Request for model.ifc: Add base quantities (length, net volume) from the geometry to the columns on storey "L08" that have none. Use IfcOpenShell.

First a look at what the model holds.

```python
import ifcopenshell
import ifcopenshell.util.element
import ifcopenshell.util.unit

model = ifcopenshell.open("model.ifc")
print(model.schema)
for unit_type in ("LENGTHUNIT", "AREAUNIT", "VOLUMEUNIT"):
    print(unit_type, ifcopenshell.util.unit.calculate_unit_scale(model, unit_type))
storey = next(s for s in model.by_type("IfcBuildingStorey") if s.Name == "L08")
columns = [e for e in ifcopenshell.util.element.get_decomposition(storey) if e.is_a("IfcColumn")]
for e in sorted(columns, key=lambda e: e.id()):
    print(e.id(), e.is_a(), e.Name, list(ifcopenshell.util.element.get_psets(e, qtos_only=True)), sep=" | ")
```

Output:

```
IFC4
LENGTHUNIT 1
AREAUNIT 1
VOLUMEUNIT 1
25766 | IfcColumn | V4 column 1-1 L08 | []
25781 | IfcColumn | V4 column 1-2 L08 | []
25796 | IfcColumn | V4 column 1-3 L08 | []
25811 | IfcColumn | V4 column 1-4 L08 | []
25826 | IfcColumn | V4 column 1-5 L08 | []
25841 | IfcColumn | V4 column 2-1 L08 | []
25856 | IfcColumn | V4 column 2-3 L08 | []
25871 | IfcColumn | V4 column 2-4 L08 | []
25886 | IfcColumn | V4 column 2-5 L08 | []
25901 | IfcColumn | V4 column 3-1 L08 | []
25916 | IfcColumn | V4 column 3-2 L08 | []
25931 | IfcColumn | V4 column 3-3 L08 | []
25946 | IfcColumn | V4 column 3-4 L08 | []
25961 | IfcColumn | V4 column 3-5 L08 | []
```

```python
import ifcopenshell
import ifcopenshell.api.pset
import ifcopenshell.geom
import ifcopenshell.util.element
import ifcopenshell.util.shape
import ifcopenshell.util.unit

model = ifcopenshell.open("model.ifc")
unit_scale = ifcopenshell.util.unit.calculate_unit_scale(model)
volume_scale = ifcopenshell.util.unit.calculate_unit_scale(model, "VOLUMEUNIT")
settings = ifcopenshell.geom.settings()

storey = next(s for s in model.by_type("IfcBuildingStorey") if s.Name == "L08")
columns = [e for e in ifcopenshell.util.element.get_decomposition(storey) if e.is_a("IfcColumn")]

for e in sorted(columns, key=lambda e: e.id()):
    if ifcopenshell.util.element.get_psets(e, qtos_only=True, should_inherit=False):
        continue
    # Geometry comes back in metres, in the element's own axes.
    shape = ifcopenshell.geom.create_shape(settings, e)
    values = {
        "Length": ifcopenshell.util.shape.get_z(shape.geometry) / unit_scale,
        "NetVolume": ifcopenshell.util.shape.get_volume(shape.geometry) / volume_scale,
    }
    qto = ifcopenshell.api.pset.add_qto(model, product=e, name="Qto_ColumnBaseQuantities")
    ifcopenshell.api.pset.edit_qto(model, qto=qto, properties=values)
    print(e.id(), {k: round(v, 3) for k, v in values.items()})

model.write("model_edited.ifc")
```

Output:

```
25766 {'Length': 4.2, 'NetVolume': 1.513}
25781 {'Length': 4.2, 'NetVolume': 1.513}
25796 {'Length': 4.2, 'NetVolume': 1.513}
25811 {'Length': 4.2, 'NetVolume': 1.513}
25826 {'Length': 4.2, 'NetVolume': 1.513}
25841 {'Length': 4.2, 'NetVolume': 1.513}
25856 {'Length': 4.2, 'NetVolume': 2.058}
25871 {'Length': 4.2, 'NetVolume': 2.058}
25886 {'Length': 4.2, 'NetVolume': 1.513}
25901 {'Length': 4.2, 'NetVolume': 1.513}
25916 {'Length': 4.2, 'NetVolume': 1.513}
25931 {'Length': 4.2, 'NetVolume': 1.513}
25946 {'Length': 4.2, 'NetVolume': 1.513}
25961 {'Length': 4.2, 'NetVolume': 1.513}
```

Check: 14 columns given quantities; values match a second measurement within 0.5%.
